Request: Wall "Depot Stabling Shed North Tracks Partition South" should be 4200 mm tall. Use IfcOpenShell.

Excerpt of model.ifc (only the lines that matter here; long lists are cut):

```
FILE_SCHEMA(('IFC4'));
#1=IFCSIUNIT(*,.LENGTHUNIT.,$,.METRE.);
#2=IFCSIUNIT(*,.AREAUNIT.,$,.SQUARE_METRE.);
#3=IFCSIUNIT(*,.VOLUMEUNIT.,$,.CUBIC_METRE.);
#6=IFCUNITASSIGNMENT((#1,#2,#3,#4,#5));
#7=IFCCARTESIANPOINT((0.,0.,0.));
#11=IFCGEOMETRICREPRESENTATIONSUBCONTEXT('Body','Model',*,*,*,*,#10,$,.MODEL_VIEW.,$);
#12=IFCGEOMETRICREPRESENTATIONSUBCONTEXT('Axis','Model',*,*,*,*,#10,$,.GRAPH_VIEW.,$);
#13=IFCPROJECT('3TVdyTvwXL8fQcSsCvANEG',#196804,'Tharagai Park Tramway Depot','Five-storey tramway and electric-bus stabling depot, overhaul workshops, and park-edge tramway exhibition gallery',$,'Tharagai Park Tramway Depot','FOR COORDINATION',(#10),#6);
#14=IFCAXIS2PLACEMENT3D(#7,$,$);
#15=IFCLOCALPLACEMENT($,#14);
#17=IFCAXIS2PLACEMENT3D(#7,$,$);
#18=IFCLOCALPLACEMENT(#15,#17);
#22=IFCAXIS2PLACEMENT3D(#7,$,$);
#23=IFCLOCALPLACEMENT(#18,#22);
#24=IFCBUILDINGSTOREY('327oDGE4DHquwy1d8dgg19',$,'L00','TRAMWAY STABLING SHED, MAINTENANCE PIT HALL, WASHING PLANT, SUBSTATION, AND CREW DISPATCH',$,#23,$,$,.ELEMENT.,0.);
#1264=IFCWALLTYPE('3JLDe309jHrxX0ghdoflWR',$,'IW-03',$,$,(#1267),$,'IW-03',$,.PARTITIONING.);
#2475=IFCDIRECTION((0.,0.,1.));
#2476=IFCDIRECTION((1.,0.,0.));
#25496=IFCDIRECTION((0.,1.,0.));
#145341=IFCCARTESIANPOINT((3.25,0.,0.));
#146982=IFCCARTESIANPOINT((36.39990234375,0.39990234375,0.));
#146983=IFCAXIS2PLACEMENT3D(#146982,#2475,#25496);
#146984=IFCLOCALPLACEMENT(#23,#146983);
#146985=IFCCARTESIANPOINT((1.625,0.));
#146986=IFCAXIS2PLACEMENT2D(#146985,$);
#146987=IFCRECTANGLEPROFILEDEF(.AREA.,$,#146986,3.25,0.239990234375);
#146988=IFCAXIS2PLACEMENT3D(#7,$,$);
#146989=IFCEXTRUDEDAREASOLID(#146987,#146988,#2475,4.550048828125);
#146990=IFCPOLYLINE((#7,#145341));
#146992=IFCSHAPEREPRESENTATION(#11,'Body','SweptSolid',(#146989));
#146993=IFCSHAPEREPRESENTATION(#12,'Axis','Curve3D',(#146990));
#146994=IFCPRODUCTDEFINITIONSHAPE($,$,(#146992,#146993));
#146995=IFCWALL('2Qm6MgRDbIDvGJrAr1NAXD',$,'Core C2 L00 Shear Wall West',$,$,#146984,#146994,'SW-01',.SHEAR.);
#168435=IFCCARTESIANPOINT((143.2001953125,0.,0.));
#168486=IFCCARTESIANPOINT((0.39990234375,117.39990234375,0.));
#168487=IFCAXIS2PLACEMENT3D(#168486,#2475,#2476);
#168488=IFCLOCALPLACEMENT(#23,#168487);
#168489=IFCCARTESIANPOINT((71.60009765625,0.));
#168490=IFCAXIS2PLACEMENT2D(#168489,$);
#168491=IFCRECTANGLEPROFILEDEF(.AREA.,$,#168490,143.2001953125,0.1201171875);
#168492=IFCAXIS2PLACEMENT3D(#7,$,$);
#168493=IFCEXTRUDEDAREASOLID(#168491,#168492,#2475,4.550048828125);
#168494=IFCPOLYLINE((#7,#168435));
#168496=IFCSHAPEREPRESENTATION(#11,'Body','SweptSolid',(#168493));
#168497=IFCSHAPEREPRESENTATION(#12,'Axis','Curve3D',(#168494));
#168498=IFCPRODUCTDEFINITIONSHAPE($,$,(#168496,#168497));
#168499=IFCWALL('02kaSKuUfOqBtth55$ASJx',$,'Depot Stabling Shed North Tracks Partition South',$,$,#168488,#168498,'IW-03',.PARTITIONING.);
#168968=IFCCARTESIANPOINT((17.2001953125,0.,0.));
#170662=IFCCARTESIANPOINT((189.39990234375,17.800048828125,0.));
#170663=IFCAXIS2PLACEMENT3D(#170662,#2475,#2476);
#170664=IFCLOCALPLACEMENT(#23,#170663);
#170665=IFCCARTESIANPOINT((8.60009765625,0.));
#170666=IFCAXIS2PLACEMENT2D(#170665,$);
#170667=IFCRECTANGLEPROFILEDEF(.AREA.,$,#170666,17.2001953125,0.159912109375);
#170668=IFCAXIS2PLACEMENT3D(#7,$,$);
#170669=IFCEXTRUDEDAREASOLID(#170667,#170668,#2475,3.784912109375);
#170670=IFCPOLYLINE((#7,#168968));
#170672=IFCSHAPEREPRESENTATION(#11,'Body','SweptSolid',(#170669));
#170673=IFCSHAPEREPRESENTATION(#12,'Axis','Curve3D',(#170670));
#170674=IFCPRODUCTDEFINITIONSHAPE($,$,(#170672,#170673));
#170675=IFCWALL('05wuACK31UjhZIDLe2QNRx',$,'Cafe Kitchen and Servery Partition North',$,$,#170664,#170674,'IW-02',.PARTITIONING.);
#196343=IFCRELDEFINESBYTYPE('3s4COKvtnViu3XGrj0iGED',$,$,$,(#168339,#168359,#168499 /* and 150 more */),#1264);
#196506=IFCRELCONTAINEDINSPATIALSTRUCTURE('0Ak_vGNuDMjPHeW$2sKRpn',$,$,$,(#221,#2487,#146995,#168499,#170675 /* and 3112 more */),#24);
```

```python
import ifcopenshell
import ifcopenshell.geom
import ifcopenshell.util.representation
import ifcopenshell.util.shape
import ifcopenshell.util.unit

model = ifcopenshell.open("model.ifc")
unit_scale = ifcopenshell.util.unit.calculate_unit_scale(model)
settings = ifcopenshell.geom.settings()


def volume(element):
    """Net volume in cubic metres, openings subtracted."""
    shape = ifcopenshell.geom.create_shape(settings, element)
    return ifcopenshell.util.shape.get_volume(shape.geometry)


wall = model.by_guid("02kaSKuUfOqBtth55$ASJx")
before = volume(wall)

body = ifcopenshell.util.representation.get_representation(wall, "Model", "Body")
solid = body.Items[0]
old_height = solid.Depth
solid.Depth = 4.2 / unit_scale
after = volume(wall)

print(f"height {old_height:g} -> {solid.Depth:g}, volume {before:.3f} -> {after:.3f} m3")

model.write("model_edited.ifc")
```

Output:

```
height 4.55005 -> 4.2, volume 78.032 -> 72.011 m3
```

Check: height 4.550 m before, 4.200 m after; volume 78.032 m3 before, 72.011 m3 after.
